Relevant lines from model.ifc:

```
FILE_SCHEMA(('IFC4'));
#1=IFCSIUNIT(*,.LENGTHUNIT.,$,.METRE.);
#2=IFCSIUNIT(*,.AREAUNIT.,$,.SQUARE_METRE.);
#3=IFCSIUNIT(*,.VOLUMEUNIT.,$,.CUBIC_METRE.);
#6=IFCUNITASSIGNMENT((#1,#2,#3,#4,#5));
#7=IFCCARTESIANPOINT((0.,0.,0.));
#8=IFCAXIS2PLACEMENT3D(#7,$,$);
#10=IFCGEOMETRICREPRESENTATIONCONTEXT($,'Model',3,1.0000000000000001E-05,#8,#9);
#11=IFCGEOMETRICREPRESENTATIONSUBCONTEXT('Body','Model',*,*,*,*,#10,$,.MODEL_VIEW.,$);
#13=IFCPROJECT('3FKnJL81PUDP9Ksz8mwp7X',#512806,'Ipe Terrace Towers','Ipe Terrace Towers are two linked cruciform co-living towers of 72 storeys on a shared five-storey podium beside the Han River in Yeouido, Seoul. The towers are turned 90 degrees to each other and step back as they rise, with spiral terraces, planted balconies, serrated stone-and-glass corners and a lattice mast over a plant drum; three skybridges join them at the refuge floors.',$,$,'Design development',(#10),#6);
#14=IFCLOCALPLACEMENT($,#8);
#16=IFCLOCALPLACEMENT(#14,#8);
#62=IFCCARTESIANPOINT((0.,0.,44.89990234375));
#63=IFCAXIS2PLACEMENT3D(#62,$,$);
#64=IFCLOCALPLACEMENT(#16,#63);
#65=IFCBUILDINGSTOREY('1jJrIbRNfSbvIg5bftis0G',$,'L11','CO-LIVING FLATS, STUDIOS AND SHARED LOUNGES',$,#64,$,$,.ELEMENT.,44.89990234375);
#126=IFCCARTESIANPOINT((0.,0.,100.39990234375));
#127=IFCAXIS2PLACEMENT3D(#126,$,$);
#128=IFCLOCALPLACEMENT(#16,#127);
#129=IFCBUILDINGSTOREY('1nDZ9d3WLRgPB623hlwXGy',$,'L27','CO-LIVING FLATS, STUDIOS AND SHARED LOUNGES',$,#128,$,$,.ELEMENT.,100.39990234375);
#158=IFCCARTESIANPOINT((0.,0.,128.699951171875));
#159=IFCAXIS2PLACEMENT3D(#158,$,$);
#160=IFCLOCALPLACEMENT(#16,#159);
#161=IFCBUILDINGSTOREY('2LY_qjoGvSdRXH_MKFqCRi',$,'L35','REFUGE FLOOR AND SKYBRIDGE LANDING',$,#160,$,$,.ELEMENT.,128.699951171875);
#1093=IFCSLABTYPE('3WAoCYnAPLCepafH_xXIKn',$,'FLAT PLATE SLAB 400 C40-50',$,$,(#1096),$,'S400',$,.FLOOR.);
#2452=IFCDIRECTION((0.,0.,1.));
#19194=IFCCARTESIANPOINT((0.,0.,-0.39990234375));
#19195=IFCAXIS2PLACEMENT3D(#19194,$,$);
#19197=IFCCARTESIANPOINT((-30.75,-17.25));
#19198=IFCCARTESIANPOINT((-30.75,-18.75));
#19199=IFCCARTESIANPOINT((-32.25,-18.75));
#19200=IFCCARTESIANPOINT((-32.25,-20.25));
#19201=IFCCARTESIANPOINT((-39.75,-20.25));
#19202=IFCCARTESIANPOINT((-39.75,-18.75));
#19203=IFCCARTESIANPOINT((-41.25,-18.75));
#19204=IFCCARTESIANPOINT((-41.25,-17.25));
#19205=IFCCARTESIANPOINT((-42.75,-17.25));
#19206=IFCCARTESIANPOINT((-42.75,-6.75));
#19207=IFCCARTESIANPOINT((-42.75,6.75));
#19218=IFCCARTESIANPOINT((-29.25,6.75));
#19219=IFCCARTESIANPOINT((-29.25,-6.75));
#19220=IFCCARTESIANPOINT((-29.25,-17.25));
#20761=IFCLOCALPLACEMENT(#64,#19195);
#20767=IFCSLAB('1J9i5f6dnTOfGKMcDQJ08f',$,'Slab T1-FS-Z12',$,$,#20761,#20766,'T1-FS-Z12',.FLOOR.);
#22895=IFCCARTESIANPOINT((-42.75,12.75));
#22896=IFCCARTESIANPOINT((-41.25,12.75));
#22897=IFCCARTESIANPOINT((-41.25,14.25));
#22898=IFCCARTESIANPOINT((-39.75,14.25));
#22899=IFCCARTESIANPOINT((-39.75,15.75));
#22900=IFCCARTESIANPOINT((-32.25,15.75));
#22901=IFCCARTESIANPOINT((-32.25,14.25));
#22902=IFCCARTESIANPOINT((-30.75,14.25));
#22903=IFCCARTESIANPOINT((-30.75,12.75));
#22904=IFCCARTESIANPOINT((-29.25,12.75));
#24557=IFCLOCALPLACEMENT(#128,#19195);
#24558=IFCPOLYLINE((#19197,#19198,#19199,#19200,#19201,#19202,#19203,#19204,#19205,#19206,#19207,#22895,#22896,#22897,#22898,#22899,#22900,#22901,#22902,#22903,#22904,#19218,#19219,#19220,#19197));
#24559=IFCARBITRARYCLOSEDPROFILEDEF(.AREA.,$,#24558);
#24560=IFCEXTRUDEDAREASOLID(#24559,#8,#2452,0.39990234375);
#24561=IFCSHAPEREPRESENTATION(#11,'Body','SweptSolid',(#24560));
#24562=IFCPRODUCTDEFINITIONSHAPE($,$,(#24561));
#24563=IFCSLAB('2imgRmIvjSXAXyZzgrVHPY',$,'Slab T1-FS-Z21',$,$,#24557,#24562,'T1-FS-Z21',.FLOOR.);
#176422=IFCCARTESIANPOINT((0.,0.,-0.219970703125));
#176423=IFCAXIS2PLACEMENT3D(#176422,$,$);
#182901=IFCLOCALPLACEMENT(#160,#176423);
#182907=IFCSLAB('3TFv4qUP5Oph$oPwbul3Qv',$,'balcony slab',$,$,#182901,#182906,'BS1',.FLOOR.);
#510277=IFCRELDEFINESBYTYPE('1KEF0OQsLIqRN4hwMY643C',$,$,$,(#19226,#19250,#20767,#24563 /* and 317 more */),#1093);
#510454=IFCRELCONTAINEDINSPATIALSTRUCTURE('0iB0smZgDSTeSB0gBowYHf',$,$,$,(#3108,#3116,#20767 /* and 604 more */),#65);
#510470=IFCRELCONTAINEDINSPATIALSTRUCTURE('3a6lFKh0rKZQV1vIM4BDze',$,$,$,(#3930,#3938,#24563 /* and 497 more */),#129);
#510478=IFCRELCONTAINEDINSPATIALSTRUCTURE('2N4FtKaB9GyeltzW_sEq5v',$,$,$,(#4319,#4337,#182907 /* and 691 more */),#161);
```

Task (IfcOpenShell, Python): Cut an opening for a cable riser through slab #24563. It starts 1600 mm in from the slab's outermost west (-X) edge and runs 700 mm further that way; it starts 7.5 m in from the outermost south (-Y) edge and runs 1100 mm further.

```python
import numpy as np
import ifcopenshell
import ifcopenshell.api.feature
import ifcopenshell.api.geometry
import ifcopenshell.api.root
import ifcopenshell.geom
import ifcopenshell.util.placement
import ifcopenshell.util.representation
import ifcopenshell.util.shape
import ifcopenshell.util.unit

model = ifcopenshell.open("model.ifc")
unit_scale = ifcopenshell.util.unit.calculate_unit_scale(model)
settings = ifcopenshell.geom.settings()


def volume(element):
    """Net volume in cubic metres, openings subtracted."""
    shape = ifcopenshell.geom.create_shape(settings, element)
    return ifcopenshell.util.shape.get_volume(shape.geometry)


slab = model.by_guid("2imgRmIvjSXAXyZzgrVHPY")
before = volume(slab)

# Extent in the slab's own axes, in metres. The edges named are its -X and -Y sides.
slab_shape = ifcopenshell.geom.create_shape(settings, slab)
vertices = ifcopenshell.util.shape.get_vertices(slab_shape.geometry)
x_min, y_min, bottom = vertices.min(axis=0)
top = vertices[:, 2].max()

opening = ifcopenshell.api.root.create_entity(model, ifc_class="IfcOpeningElement", name="Cable riser opening", predefined_type="OPENING")
context = ifcopenshell.util.representation.get_context(model, "Model", "Body", "MODEL_VIEW")
width, depth = 0.7, 1.1
outline = [(0.0, 0.0), (width, 0.0), (width, depth), (0.0, depth), (0.0, 0.0)]
# Overshoot both faces by 50 mm so the cut is clean.
shape = ifcopenshell.api.geometry.add_slab_representation(
    model, context=context, depth=top - bottom + 0.1, polyline=outline
)
ifcopenshell.api.geometry.assign_representation(model, product=opening, representation=shape)

matrix = ifcopenshell.util.placement.get_local_placement(slab.ObjectPlacement)
matrix[:, 3] = matrix @ np.append(np.array([x_min + 1.6, y_min + 7.5, bottom - 0.05]) / unit_scale, 1.0)
ifcopenshell.api.geometry.edit_object_placement(model, product=opening, matrix=matrix, is_si=False)
ifcopenshell.api.feature.add_feature(model, feature=opening, element=slab)

after = volume(slab)

print(f"slab volume {before:.3f} -> {after:.3f} m3")

model.write("model_edited.ifc")
```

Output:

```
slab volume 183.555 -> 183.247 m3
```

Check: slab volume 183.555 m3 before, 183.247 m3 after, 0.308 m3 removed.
